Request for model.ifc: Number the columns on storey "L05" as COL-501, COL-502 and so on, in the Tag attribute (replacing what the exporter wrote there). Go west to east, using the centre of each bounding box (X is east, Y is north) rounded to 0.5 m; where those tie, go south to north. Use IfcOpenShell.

First a look at what the model holds.

```python
import ifcopenshell
import ifcopenshell.util.element
import ifcopenshell.util.placement

model = ifcopenshell.open("model.ifc")
print(model.schema)
storey = next(s for s in model.by_type("IfcBuildingStorey") if s.Name == "L05")
columns = [e for e in ifcopenshell.util.element.get_decomposition(storey) if e.is_a("IfcColumn")]
for e in sorted(columns, key=lambda e: e.id()):
    origin = ifcopenshell.util.placement.get_local_placement(e.ObjectPlacement)[:3, 3]
    print(e.id(), e.Tag, e.Name, origin.round(2) + 0.0, sep=" | ")
```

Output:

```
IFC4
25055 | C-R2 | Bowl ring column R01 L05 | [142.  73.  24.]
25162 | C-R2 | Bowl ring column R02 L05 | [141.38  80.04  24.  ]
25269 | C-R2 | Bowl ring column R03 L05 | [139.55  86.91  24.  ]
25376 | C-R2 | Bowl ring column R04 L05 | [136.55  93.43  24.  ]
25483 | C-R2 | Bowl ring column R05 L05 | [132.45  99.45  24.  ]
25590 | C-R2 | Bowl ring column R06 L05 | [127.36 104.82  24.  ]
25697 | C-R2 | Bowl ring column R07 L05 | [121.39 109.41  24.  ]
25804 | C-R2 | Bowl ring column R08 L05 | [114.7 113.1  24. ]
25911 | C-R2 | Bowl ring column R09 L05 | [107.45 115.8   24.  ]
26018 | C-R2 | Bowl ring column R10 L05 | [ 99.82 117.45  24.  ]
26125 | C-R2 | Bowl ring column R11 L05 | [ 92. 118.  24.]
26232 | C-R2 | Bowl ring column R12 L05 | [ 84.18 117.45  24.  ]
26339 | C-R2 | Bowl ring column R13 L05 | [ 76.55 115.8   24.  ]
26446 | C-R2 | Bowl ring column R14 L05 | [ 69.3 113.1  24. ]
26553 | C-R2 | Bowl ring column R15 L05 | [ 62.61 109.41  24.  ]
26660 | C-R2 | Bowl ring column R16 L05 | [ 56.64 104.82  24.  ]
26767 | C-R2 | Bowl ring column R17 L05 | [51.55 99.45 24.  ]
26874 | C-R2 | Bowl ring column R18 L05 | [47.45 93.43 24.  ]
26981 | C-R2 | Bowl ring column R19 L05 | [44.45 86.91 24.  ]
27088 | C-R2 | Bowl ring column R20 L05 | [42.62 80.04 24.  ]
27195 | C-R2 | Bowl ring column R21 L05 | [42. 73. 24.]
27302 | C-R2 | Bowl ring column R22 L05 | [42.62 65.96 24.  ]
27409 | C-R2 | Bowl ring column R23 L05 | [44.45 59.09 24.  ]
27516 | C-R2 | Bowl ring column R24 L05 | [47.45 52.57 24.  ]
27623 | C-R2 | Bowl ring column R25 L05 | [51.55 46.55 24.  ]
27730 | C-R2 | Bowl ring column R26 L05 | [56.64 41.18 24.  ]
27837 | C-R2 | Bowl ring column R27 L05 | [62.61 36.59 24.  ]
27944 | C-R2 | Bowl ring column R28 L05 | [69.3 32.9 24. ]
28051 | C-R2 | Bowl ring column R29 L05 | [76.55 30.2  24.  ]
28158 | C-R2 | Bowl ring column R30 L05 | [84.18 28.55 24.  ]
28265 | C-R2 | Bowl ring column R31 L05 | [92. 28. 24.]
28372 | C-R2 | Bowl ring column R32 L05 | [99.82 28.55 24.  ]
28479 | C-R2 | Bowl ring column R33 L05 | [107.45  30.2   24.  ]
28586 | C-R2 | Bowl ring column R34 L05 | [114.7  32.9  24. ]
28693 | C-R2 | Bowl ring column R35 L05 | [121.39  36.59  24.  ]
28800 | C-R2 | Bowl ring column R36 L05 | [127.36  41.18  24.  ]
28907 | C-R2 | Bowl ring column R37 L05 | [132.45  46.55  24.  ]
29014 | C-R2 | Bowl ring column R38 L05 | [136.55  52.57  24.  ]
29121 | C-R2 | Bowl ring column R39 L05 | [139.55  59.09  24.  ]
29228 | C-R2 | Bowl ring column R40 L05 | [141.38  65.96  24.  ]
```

```python
import ifcopenshell
import ifcopenshell.geom
import ifcopenshell.util.element
import ifcopenshell.util.shape

model = ifcopenshell.open("model.ifc")
settings = ifcopenshell.geom.settings()
settings.set("use-world-coords", True)


def centre(element):
    shape = ifcopenshell.geom.create_shape(settings, element)
    return ifcopenshell.util.shape.get_bbox_centroid(shape.geometry)


storey = next(s for s in model.by_type("IfcBuildingStorey") if s.Name == "L05")
columns = [e for e in ifcopenshell.util.element.get_decomposition(storey) if e.is_a("IfcColumn")]

# Insertion points can sit at a corner or the storey origin, so sort by the geometry (in metres).
centres = {e: centre(e) for e in columns}
columns.sort(key=lambda e: (round(centres[e][0] / 0.5), centres[e][1]))

for i, e in enumerate(columns, start=1):
    number = f"COL-5{i:02d}"
    e.Tag = number
    print(e.id(), number)

model.write("model_updated.ifc")
```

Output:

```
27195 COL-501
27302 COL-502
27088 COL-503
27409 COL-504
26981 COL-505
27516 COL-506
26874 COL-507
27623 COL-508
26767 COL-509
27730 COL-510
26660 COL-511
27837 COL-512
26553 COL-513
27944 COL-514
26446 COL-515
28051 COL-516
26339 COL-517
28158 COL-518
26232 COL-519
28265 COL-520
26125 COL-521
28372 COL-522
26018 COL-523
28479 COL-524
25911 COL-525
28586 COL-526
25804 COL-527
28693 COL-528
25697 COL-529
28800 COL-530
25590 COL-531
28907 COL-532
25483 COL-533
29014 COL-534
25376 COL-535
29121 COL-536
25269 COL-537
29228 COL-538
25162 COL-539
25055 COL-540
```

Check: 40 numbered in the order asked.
